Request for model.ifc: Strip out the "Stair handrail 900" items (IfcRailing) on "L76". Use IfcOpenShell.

First a look at what the model holds.

```python
import ifcopenshell
import ifcopenshell.util.element

model = ifcopenshell.open("model.ifc")
print(model.schema)
storey = next(s for s in model.by_type("IfcBuildingStorey") if s.Name == "L76")
railings = [e for e in ifcopenshell.util.element.get_decomposition(storey) if e.is_a("IfcRailing")]
seen = {}
for e in railings:
    element_type = ifcopenshell.util.element.get_type(e)
    name = element_type.Name if element_type not in (None, e) else None
    seen[name] = seen.get(name, 0) + 1
for name, count in sorted(seen.items(), key=str):
    print(count, "x", name)
```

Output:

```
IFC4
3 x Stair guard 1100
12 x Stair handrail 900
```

```python
import ifcopenshell
import ifcopenshell.api.root
import ifcopenshell.util.element

model = ifcopenshell.open("model.ifc")

storey = next(s for s in model.by_type("IfcBuildingStorey") if s.Name == "L76")
railings = [e for e in ifcopenshell.util.element.get_decomposition(storey) if e.is_a("IfcRailing")]
targets = [e for e in railings if (t := ifcopenshell.util.element.get_type(e)) not in (None, e) and t.Name == "Stair handrail 900"]

for e in targets:
    ifcopenshell.api.root.remove_product(model, product=e)
print(len(targets), "removed")

model.write("model_edited.ifc")
```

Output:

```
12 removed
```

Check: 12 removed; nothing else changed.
